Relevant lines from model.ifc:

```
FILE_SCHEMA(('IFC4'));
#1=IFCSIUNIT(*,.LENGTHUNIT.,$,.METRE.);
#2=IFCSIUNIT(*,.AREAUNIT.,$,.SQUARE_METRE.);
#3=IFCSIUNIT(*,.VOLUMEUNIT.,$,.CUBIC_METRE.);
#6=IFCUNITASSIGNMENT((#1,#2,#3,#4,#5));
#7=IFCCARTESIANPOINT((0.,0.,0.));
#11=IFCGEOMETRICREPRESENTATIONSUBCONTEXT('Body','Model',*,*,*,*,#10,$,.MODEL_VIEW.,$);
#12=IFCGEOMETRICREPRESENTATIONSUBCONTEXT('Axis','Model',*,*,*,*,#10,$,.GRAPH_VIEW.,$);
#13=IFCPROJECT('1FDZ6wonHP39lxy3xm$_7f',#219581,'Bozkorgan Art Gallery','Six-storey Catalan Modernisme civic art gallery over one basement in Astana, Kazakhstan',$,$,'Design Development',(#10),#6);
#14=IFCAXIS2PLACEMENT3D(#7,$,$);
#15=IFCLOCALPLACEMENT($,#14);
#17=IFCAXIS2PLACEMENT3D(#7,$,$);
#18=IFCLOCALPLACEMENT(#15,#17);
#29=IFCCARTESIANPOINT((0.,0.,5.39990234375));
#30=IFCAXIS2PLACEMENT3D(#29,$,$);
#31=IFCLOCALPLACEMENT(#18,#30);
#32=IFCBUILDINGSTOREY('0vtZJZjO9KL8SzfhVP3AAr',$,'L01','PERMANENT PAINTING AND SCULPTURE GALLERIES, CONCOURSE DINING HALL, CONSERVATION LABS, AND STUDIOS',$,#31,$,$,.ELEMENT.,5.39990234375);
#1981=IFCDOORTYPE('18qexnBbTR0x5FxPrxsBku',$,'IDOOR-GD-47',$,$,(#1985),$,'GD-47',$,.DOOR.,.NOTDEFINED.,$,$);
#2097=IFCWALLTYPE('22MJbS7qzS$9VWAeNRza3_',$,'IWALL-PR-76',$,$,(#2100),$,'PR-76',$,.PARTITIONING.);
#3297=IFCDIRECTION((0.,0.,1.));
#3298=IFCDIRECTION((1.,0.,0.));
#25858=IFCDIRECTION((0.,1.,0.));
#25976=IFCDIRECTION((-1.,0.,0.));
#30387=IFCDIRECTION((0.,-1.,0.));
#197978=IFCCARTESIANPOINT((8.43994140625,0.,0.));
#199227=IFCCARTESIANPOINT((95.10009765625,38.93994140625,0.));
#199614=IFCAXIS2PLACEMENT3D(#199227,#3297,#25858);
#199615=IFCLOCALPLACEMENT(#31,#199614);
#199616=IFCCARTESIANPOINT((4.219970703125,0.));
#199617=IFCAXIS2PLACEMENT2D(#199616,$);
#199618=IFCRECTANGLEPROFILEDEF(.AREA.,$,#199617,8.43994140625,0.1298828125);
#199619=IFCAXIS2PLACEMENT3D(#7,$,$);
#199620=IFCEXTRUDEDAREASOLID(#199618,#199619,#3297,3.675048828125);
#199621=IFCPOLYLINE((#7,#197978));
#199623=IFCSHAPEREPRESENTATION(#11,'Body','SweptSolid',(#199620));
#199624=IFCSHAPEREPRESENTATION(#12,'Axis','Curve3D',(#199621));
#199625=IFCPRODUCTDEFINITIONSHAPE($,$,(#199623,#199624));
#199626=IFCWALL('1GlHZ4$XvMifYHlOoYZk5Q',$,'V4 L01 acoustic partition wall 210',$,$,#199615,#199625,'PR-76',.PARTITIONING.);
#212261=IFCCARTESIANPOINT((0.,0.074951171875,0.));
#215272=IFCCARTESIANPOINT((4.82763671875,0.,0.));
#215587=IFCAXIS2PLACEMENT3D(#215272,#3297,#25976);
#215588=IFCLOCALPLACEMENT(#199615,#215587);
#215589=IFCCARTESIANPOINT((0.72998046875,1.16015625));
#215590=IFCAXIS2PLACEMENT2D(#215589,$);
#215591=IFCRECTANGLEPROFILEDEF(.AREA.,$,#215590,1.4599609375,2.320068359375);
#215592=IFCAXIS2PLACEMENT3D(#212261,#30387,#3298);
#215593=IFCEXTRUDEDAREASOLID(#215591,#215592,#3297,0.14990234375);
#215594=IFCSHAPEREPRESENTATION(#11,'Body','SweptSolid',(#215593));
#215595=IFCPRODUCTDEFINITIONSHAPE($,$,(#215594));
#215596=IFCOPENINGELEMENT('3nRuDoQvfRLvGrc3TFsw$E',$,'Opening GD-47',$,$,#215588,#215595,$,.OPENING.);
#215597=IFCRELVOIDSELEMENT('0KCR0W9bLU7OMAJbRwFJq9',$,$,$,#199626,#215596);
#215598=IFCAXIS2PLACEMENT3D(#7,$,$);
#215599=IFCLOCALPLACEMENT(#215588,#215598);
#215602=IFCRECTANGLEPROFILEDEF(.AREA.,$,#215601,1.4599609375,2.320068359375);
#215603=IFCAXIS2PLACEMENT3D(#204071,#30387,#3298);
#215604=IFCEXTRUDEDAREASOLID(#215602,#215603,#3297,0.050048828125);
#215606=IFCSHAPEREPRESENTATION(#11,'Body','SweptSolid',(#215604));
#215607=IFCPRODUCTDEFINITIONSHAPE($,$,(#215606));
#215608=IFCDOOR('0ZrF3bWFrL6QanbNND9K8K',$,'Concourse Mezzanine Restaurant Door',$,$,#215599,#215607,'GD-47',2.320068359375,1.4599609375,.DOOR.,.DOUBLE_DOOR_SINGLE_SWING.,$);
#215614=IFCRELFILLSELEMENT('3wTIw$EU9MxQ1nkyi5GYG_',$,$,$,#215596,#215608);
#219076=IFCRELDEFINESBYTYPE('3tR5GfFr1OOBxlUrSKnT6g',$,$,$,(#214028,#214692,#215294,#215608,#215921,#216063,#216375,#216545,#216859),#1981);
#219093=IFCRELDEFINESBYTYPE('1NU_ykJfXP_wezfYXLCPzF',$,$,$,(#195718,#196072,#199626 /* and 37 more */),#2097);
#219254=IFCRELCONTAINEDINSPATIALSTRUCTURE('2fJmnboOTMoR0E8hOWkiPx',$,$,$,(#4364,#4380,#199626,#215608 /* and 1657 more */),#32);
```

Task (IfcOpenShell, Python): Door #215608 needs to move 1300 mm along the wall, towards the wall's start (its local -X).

```python
import ifcopenshell
import ifcopenshell.api.geometry
import ifcopenshell.util.placement

model = ifcopenshell.open("model.ifc")

door = model.by_guid("0ZrF3bWFrL6QanbNND9K8K")
opening = door.FillsVoids[0].RelatingOpeningElement
wall = opening.VoidsElements[0].RelatingBuildingElement

wall_matrix = ifcopenshell.util.placement.get_local_placement(wall.ObjectPlacement)
shift = wall_matrix[:3, 0] * -1.3
before = ifcopenshell.util.placement.get_local_placement(door.ObjectPlacement)[:3, 3].copy()

# The door is placed relative to its opening, so it follows when the opening moves.
matrix = ifcopenshell.util.placement.get_local_placement(opening.ObjectPlacement)
matrix[:3, 3] += shift
ifcopenshell.api.geometry.edit_object_placement(
    model, product=opening, matrix=matrix, is_si=False, should_transform_children=True
)

after = ifcopenshell.util.placement.get_local_placement(door.ObjectPlacement)[:3, 3]
print("door moved by", (after - before).round(3) + 0.0)

model.write("model-out.ifc")
```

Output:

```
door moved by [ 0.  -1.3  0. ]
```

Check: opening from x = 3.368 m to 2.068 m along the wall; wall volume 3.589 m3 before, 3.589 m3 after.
